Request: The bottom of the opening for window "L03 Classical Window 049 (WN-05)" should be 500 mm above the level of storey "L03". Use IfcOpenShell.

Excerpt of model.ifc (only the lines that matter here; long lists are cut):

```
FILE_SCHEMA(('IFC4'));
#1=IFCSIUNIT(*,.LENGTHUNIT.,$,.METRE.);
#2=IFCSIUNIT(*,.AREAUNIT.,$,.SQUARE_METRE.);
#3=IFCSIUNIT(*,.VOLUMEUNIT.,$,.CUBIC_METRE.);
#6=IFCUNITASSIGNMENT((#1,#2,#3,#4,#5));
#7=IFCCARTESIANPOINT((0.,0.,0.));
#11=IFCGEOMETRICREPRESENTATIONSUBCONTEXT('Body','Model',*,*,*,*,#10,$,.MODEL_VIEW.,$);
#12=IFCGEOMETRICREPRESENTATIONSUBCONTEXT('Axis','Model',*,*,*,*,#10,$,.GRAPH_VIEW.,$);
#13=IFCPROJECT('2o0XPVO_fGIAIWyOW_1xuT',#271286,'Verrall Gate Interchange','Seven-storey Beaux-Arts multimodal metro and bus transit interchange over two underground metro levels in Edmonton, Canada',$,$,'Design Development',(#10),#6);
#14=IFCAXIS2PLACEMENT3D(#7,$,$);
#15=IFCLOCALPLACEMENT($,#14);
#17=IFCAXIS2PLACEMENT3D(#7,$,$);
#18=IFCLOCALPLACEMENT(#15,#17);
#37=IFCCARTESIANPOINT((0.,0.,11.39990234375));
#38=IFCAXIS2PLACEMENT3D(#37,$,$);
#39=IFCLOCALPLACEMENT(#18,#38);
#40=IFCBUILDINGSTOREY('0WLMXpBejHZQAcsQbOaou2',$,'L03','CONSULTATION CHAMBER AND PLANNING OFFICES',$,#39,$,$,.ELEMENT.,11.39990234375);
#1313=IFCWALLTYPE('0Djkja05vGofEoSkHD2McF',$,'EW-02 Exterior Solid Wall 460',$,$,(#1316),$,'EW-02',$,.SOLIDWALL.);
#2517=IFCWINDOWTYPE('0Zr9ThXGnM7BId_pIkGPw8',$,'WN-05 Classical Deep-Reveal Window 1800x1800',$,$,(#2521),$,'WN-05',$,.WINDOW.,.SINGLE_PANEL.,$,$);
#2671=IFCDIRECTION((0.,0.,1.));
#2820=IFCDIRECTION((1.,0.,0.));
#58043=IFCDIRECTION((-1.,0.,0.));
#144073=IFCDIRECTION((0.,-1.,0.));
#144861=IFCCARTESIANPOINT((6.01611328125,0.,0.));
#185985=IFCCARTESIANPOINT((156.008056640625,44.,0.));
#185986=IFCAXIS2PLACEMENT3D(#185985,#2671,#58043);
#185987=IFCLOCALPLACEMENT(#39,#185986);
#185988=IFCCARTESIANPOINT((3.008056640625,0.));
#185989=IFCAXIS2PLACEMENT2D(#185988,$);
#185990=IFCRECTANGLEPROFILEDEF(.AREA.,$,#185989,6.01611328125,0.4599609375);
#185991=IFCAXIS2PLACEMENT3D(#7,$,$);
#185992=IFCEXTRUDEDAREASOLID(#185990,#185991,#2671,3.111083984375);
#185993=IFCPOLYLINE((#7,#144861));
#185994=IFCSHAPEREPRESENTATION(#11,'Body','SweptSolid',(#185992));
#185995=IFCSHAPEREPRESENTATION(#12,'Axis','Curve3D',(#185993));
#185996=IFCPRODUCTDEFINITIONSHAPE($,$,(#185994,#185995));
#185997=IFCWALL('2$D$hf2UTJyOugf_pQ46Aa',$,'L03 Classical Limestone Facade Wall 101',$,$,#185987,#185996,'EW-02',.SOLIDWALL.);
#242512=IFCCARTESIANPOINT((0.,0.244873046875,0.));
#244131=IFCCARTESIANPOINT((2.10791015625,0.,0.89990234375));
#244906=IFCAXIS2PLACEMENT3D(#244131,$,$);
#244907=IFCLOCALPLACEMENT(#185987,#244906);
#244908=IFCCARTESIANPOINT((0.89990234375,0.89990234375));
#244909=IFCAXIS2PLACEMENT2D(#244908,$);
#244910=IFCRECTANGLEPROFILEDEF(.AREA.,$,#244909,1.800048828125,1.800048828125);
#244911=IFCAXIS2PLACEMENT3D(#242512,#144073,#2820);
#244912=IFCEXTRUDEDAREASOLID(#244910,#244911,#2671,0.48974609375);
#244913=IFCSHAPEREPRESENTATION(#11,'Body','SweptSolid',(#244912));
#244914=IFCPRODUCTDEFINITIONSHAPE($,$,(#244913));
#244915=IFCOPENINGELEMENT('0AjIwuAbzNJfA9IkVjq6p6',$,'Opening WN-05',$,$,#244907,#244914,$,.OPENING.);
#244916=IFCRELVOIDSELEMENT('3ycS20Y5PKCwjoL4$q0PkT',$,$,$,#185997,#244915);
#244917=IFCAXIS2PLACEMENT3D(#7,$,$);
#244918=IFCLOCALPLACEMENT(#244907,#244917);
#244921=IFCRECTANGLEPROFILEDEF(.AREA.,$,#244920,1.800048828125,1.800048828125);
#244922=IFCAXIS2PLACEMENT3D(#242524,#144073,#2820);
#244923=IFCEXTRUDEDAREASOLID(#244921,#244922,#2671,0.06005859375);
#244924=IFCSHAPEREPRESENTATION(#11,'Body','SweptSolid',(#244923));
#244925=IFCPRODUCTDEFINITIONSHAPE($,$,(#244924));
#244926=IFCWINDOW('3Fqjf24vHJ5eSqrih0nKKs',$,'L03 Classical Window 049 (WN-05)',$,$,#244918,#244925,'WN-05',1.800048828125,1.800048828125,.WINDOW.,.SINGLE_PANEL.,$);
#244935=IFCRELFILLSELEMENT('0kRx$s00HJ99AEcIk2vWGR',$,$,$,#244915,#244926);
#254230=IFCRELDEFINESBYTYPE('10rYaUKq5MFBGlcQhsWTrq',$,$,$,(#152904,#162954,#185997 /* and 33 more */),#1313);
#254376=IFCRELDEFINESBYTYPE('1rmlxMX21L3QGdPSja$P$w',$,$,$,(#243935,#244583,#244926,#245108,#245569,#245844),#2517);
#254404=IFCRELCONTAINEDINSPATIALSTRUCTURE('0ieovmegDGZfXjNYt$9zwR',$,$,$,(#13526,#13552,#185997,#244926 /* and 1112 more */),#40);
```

```python
import numpy as np
import ifcopenshell
import ifcopenshell.api.geometry
import ifcopenshell.geom
import ifcopenshell.util.element
import ifcopenshell.util.placement
import ifcopenshell.util.shape
import ifcopenshell.util.unit

model = ifcopenshell.open("model.ifc")
unit_scale = ifcopenshell.util.unit.calculate_unit_scale(model)

window = model.by_id(244926)
opening = window.FillsVoids[0].RelatingOpeningElement
storey = ifcopenshell.util.element.get_container(window, ifc_class="IfcBuildingStorey")
level = ifcopenshell.util.placement.get_local_placement(storey.ObjectPlacement)[2, 3]

# The opening's origin need not be at the sill, so measure its lowest point.
shape = ifcopenshell.geom.create_shape(ifcopenshell.geom.settings(), opening)
bottom = ifcopenshell.util.shape.get_shape_bottom_elevation(shape, shape.geometry) / unit_scale
dz = level + 0.5 - bottom

shift = np.array([0.0, 0.0, dz])
# The window is placed relative to its opening, so it follows when the opening moves.
matrix = ifcopenshell.util.placement.get_local_placement(opening.ObjectPlacement)
matrix[:3, 3] += shift
ifcopenshell.api.geometry.edit_object_placement(
    model, product=opening, matrix=matrix, is_si=False, should_transform_children=True
)

print(f"moved by {dz * unit_scale:+.3f} m")

model.write("model-out.ifc")
```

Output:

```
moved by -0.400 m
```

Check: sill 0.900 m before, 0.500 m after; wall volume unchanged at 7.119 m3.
